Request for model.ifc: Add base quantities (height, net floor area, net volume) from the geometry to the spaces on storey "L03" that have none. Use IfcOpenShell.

First a look at what the model holds.

```python
import ifcopenshell
import ifcopenshell.util.element
import ifcopenshell.util.unit

model = ifcopenshell.open("model.ifc")
print(model.schema)
for unit_type in ("LENGTHUNIT", "AREAUNIT", "VOLUMEUNIT"):
    print(unit_type, ifcopenshell.util.unit.calculate_unit_scale(model, unit_type))
storey = next(s for s in model.by_type("IfcBuildingStorey") if s.Name == "L03")
spaces = [e for e in ifcopenshell.util.element.get_decomposition(storey) if e.is_a("IfcSpace")]
for e in sorted(spaces, key=lambda e: e.id()):
    print(e.id(), e.is_a(), e.Name, list(ifcopenshell.util.element.get_psets(e, qtos_only=True)), sep=" | ")
```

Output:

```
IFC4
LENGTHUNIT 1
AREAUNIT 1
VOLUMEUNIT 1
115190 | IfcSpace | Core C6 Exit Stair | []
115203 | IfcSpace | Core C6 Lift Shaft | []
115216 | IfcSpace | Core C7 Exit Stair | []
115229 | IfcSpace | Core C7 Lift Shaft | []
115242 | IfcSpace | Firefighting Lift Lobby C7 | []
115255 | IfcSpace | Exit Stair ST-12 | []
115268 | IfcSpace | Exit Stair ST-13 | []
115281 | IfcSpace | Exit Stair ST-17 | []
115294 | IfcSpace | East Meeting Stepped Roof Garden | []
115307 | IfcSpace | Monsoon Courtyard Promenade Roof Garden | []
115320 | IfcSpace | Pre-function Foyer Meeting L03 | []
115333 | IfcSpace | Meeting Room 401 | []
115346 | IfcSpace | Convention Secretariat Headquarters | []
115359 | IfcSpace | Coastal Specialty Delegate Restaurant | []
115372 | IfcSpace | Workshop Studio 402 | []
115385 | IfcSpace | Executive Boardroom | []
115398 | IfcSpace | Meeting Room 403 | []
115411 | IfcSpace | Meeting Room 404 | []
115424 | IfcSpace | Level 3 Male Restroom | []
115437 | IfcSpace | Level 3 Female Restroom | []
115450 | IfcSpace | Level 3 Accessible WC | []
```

```python
import ifcopenshell
import ifcopenshell.api.pset
import ifcopenshell.geom
import ifcopenshell.util.element
import ifcopenshell.util.shape
import ifcopenshell.util.unit

model = ifcopenshell.open("model.ifc")
unit_scale = ifcopenshell.util.unit.calculate_unit_scale(model)
area_scale = ifcopenshell.util.unit.calculate_unit_scale(model, "AREAUNIT")
volume_scale = ifcopenshell.util.unit.calculate_unit_scale(model, "VOLUMEUNIT")
settings = ifcopenshell.geom.settings()

storey = next(s for s in model.by_type("IfcBuildingStorey") if s.Name == "L03")
spaces = [e for e in ifcopenshell.util.element.get_decomposition(storey) if e.is_a("IfcSpace")]

for e in sorted(spaces, key=lambda e: e.id()):
    if ifcopenshell.util.element.get_psets(e, qtos_only=True, should_inherit=False):
        continue
    # Geometry comes back in metres, in the element's own axes.
    shape = ifcopenshell.geom.create_shape(settings, e)
    values = {
        "Height": ifcopenshell.util.shape.get_z(shape.geometry) / unit_scale,
        "NetFloorArea": ifcopenshell.util.shape.get_footprint_area(shape.geometry) / area_scale,
        "NetVolume": ifcopenshell.util.shape.get_volume(shape.geometry) / volume_scale,
    }
    qto = ifcopenshell.api.pset.add_qto(model, product=e, name="Qto_SpaceBaseQuantities")
    ifcopenshell.api.pset.edit_qto(model, qto=qto, properties=values)
    print(e.id(), {k: round(v, 3) for k, v in values.items()})

model.write("model_v2.ifc")
```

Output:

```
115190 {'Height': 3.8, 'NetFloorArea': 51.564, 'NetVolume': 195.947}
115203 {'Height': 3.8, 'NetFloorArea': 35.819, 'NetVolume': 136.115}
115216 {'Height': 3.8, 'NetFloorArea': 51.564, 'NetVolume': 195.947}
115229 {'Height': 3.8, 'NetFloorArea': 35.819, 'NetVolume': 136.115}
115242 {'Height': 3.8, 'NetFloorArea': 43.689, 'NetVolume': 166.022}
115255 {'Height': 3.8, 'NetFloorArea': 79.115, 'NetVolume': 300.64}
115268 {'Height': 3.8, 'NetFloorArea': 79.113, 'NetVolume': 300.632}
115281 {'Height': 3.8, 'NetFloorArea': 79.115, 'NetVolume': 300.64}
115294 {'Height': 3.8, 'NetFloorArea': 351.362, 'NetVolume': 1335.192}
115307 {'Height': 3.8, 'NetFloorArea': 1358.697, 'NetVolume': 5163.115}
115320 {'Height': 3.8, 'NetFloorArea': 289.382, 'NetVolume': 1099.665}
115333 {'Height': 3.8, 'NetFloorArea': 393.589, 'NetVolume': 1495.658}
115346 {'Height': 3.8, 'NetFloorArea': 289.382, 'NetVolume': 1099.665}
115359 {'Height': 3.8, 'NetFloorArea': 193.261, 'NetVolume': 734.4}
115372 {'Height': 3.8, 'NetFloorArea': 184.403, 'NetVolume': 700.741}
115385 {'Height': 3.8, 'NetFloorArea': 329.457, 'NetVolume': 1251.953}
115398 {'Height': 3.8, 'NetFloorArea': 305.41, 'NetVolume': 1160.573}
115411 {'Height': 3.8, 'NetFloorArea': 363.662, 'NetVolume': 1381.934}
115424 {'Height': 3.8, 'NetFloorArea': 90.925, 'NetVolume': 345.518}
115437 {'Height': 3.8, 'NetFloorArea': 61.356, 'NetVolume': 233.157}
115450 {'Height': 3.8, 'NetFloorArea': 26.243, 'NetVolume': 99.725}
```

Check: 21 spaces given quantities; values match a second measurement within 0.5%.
